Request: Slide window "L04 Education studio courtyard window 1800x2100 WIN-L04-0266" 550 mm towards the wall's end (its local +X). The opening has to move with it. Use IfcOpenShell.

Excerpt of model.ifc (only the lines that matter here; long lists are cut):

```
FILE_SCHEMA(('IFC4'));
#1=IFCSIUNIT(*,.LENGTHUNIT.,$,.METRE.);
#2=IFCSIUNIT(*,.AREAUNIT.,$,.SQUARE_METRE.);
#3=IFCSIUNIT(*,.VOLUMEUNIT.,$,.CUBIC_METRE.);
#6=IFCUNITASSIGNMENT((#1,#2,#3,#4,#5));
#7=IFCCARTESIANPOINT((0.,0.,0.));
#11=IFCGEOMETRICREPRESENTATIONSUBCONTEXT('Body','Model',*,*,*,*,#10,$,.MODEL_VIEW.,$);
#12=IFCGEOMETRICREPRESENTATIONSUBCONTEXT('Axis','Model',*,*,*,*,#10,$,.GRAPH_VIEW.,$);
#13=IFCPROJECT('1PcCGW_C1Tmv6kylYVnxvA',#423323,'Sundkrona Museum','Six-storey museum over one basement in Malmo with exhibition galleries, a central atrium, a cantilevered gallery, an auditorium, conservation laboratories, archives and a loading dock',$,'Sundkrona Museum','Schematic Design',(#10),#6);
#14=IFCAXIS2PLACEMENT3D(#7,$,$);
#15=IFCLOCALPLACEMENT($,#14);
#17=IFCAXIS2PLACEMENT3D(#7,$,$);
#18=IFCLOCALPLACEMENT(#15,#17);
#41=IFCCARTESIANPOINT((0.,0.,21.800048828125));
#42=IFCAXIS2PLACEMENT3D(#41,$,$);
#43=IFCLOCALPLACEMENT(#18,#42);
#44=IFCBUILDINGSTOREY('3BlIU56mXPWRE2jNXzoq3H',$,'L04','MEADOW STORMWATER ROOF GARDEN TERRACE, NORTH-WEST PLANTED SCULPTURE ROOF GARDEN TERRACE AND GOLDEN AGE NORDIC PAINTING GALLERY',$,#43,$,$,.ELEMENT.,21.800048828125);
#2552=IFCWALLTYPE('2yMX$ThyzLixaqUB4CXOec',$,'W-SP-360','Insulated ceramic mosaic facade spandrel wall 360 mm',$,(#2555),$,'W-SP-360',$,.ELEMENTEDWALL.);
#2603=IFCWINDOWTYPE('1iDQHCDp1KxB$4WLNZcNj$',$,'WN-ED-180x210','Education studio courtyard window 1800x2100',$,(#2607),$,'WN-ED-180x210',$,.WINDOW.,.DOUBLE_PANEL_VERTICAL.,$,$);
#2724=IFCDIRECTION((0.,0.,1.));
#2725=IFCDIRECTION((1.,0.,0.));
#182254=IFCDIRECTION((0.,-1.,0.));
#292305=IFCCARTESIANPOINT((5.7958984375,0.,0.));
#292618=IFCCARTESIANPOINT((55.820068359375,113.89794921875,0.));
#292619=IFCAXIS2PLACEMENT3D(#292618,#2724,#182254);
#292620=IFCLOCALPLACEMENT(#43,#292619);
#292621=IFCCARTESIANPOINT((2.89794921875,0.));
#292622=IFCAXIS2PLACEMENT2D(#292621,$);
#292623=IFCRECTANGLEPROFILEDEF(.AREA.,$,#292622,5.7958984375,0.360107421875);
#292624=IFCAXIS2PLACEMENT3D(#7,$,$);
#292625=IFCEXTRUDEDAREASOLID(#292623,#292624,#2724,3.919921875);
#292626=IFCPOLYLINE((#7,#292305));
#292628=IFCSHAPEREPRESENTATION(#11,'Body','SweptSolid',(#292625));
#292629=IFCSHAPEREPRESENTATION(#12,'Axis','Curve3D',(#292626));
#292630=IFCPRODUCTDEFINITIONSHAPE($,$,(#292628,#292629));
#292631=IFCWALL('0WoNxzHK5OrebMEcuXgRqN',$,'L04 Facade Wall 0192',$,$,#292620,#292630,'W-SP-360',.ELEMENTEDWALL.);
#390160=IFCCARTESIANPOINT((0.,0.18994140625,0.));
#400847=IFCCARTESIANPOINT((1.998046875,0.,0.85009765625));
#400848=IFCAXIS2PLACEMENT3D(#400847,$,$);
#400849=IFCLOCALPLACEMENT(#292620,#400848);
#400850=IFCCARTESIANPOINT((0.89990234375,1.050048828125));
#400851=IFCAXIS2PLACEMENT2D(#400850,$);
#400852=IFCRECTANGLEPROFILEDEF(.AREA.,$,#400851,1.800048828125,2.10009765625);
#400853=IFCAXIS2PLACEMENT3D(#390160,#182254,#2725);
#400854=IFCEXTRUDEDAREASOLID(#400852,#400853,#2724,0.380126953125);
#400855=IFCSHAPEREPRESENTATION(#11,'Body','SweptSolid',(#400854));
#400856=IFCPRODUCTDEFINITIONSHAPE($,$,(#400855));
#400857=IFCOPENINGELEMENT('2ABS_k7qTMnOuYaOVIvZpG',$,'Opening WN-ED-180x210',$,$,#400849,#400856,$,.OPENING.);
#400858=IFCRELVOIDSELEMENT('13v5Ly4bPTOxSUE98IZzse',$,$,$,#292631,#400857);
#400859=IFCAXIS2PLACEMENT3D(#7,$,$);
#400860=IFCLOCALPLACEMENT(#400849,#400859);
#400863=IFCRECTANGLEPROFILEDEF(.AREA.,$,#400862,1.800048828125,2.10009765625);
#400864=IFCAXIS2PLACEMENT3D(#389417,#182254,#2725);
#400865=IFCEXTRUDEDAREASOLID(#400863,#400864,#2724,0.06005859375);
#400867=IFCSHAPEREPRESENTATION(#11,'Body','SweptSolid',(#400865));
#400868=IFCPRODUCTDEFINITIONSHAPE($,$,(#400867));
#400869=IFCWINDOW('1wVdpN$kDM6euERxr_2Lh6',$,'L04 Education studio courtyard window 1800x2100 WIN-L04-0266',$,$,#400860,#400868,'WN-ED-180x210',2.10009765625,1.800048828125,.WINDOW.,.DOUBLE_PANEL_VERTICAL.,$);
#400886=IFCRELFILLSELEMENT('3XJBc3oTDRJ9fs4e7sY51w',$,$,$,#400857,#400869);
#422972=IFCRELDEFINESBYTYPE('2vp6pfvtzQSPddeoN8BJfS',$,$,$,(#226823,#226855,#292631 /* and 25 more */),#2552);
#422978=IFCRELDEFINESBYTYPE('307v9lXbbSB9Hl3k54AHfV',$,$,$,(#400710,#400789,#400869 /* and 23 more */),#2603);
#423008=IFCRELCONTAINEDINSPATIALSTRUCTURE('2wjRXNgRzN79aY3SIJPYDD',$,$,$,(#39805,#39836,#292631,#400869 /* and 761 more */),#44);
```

```python
import ifcopenshell
import ifcopenshell.api.geometry
import ifcopenshell.util.placement

model = ifcopenshell.open("model.ifc")

window = model.by_id(400869)
opening = window.FillsVoids[0].RelatingOpeningElement
wall = opening.VoidsElements[0].RelatingBuildingElement

wall_matrix = ifcopenshell.util.placement.get_local_placement(wall.ObjectPlacement)
shift = wall_matrix[:3, 0] * 0.55
before = ifcopenshell.util.placement.get_local_placement(window.ObjectPlacement)[:3, 3].copy()

# The window is placed relative to its opening, so it follows when the opening moves.
matrix = ifcopenshell.util.placement.get_local_placement(opening.ObjectPlacement)
matrix[:3, 3] += shift
ifcopenshell.api.geometry.edit_object_placement(
    model, product=opening, matrix=matrix, is_si=False, should_transform_children=True
)

after = ifcopenshell.util.placement.get_local_placement(window.ObjectPlacement)[:3, 3]
print("window moved by", (after - before).round(3) + 0.0)

model.write("model_rev.ifc")
```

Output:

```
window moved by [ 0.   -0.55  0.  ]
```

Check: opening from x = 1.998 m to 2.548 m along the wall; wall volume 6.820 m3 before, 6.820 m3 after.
